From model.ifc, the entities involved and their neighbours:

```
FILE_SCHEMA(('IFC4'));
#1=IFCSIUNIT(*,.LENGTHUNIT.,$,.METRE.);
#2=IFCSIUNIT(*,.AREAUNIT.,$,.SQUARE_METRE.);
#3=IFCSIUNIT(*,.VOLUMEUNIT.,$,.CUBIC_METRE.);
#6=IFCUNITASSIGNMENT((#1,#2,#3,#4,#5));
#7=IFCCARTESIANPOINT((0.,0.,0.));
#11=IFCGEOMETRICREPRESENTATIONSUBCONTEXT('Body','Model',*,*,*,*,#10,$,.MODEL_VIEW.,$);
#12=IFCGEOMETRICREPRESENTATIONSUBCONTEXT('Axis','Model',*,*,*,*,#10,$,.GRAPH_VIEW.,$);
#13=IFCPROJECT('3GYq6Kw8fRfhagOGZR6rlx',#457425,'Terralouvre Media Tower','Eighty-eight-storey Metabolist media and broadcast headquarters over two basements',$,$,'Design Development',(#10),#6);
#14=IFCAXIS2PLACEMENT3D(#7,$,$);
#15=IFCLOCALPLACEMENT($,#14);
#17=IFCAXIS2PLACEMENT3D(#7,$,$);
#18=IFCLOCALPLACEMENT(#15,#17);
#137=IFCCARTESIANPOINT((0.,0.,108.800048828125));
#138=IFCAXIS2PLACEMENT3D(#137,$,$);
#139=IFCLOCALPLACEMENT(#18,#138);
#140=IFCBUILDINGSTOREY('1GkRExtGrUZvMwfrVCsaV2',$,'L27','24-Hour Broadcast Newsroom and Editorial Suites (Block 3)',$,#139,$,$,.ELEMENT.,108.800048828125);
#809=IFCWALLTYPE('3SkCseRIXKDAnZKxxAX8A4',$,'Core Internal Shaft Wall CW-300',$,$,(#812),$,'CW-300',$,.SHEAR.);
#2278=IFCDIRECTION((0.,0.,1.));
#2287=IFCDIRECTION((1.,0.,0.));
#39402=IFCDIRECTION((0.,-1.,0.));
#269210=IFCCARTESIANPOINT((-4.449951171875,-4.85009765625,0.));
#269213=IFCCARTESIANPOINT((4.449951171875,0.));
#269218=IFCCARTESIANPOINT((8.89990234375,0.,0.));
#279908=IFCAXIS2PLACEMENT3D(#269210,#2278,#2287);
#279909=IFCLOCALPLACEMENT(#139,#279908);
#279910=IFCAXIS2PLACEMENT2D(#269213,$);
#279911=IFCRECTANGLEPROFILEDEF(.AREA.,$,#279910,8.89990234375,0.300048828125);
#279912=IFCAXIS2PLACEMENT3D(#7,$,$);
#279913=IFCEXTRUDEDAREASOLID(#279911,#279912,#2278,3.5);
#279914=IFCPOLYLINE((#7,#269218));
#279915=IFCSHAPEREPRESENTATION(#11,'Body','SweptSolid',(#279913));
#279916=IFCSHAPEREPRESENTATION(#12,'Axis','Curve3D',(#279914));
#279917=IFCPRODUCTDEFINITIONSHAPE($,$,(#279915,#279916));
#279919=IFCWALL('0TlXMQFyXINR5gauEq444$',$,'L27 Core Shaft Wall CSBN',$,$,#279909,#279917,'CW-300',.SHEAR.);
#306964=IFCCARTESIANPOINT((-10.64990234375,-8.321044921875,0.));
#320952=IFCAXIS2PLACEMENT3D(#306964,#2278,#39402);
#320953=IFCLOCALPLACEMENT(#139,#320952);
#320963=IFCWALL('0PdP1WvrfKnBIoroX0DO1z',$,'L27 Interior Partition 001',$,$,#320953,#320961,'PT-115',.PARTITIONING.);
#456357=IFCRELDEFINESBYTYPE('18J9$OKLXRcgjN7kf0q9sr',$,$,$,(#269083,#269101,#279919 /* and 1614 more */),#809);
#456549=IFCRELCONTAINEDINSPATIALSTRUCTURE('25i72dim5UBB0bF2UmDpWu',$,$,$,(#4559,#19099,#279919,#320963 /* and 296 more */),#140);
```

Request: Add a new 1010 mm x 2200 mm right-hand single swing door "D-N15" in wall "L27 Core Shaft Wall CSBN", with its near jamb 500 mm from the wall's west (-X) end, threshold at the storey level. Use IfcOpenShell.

```python
import numpy as np
import ifcopenshell
import ifcopenshell.api.feature
import ifcopenshell.api.geometry
import ifcopenshell.api.root
import ifcopenshell.api.spatial
import ifcopenshell.geom
import ifcopenshell.util.element
import ifcopenshell.util.placement
import ifcopenshell.util.representation
import ifcopenshell.util.shape
import ifcopenshell.util.unit

model = ifcopenshell.open("model.ifc")
unit_scale = ifcopenshell.util.unit.calculate_unit_scale(model)
settings = ifcopenshell.geom.settings()


def volume(element):
    """Net volume in cubic metres, openings subtracted."""
    shape = ifcopenshell.geom.create_shape(settings, element)
    return ifcopenshell.util.shape.get_volume(shape.geometry)


wall = model.by_guid("0TlXMQFyXINR5gauEq444$")
storey = ifcopenshell.util.element.get_container(wall, ifc_class="IfcBuildingStorey")
context = ifcopenshell.util.representation.get_context(model, "Model", "Body", "MODEL_VIEW")
before = volume(wall)

width, height, from_end, sill = 1.01, 2.2, 0.5, 0.0  # metres

# The wall runs along its own X axis, and the end named is its -X end.
wall_shape = ifcopenshell.geom.create_shape(settings, wall)
x, y, z = ifcopenshell.util.shape.get_vertices(wall_shape.geometry).T
start = x.min() + from_end
face, thickness = float(y.min()), float(y.max() - y.min())
wall_matrix = ifcopenshell.util.placement.get_local_placement(wall.ObjectPlacement)
level = ifcopenshell.util.placement.get_local_placement(storey.ObjectPlacement)[2, 3]


def in_wall(x, y):
    """Placement at x, y metres in the wall's axes, at sill height."""
    matrix = wall_matrix.copy()
    matrix[:, 3] = wall_matrix @ np.array([x / unit_scale, y / unit_scale, 0.0, 1.0])
    matrix[2, 3] = level + sill / unit_scale
    return matrix


# Opening: a box that overshoots both wall faces by 50 mm.
opening = ifcopenshell.api.root.create_entity(model, ifc_class="IfcOpeningElement", predefined_type="OPENING")
box = ifcopenshell.api.geometry.add_wall_representation(
    model, context=context, length=width, height=height, thickness=thickness + 0.1
)
ifcopenshell.api.geometry.assign_representation(model, product=opening, representation=box)
ifcopenshell.api.geometry.edit_object_placement(model, product=opening, matrix=in_wall(start, face - 0.05), is_si=False)
ifcopenshell.api.feature.add_feature(model, feature=opening, element=wall)

door = ifcopenshell.api.root.create_entity(model, ifc_class="IfcDoor", name="D-N15", predefined_type="DOOR")
door.OverallWidth, door.OverallHeight = width / unit_scale, height / unit_scale
door.OperationType = "SINGLE_SWING_RIGHT"
body = ifcopenshell.api.geometry.add_door_representation(
    model,
    context=context,
    overall_width=door.OverallWidth,
    overall_height=door.OverallHeight,
    operation_type="SINGLE_SWING_RIGHT",
    lining_properties={"LiningDepth": thickness / unit_scale, "ThresholdDepth": thickness / unit_scale},
)
ifcopenshell.api.geometry.assign_representation(model, product=door, representation=body)
ifcopenshell.api.spatial.assign_container(model, products=[door], relating_structure=storey)
ifcopenshell.api.feature.add_filling(model, opening=opening, element=door)

# The lining spans the wall, so the door starts at the wall face.
ifcopenshell.api.geometry.edit_object_placement(model, product=door, matrix=in_wall(start, face), is_si=False)

after = volume(wall)

print(f"wall volume {before:.3f} -> {after:.3f} m3")

model.write("model-out.ifc")
```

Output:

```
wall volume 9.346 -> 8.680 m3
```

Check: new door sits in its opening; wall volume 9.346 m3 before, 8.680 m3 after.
